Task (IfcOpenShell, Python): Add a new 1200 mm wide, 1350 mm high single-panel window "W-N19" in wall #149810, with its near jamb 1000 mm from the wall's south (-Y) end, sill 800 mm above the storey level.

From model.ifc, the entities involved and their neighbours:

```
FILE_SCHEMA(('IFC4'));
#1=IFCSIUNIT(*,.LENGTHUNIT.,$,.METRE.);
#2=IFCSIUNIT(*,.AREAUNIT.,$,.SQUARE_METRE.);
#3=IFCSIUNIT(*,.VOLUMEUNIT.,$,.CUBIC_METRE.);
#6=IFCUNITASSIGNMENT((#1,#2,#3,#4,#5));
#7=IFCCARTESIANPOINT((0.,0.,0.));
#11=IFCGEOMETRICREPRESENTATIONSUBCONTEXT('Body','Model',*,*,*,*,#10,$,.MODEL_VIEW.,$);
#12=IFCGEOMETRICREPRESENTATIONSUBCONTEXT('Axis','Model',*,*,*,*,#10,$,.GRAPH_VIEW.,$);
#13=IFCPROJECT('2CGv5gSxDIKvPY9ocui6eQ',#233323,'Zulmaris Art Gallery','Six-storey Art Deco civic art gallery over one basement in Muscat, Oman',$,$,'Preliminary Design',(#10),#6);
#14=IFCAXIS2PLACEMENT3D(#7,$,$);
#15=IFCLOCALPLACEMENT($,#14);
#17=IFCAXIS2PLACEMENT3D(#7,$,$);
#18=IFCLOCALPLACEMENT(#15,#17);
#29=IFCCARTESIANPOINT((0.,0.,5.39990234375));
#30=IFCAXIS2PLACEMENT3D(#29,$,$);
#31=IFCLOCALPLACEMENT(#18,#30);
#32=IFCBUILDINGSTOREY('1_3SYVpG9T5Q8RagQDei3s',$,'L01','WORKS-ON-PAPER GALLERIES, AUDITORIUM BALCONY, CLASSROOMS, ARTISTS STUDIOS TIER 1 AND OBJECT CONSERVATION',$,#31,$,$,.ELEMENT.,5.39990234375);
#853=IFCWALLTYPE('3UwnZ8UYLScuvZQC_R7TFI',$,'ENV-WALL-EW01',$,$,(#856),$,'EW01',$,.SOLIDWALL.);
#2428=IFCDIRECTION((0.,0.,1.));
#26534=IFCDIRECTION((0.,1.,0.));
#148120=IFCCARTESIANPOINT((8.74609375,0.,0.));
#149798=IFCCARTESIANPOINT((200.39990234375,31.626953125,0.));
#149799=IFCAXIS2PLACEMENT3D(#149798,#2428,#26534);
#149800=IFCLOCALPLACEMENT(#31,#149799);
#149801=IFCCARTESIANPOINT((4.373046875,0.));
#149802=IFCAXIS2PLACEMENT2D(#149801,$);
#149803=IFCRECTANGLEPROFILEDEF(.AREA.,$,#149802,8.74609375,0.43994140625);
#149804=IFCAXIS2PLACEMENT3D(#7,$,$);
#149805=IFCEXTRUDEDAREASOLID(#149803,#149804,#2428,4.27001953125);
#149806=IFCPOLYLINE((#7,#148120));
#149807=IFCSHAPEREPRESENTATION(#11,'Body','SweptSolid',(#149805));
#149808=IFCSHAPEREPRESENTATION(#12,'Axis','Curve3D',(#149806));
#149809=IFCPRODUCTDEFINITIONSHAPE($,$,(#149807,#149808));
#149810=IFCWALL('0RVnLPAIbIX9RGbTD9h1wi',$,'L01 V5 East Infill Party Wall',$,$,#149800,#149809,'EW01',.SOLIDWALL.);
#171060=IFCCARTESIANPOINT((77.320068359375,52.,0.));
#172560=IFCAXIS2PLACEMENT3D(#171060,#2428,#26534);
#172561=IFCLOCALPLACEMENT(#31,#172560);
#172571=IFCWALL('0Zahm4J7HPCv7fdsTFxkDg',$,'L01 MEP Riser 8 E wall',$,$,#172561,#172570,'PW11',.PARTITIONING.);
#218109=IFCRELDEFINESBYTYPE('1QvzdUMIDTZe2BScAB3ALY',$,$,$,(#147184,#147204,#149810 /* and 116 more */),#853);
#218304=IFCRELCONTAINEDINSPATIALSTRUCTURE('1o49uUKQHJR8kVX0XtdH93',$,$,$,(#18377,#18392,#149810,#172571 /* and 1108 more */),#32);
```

```python
import numpy as np
import ifcopenshell
import ifcopenshell.api.feature
import ifcopenshell.api.geometry
import ifcopenshell.api.root
import ifcopenshell.api.spatial
import ifcopenshell.geom
import ifcopenshell.util.element
import ifcopenshell.util.placement
import ifcopenshell.util.representation
import ifcopenshell.util.shape
import ifcopenshell.util.unit

model = ifcopenshell.open("model.ifc")
unit_scale = ifcopenshell.util.unit.calculate_unit_scale(model)
settings = ifcopenshell.geom.settings()


def volume(element):
    """Net volume in cubic metres, openings subtracted."""
    shape = ifcopenshell.geom.create_shape(settings, element)
    return ifcopenshell.util.shape.get_volume(shape.geometry)


wall = model.by_id(149810)
storey = ifcopenshell.util.element.get_container(wall, ifc_class="IfcBuildingStorey")
context = ifcopenshell.util.representation.get_context(model, "Model", "Body", "MODEL_VIEW")
before = volume(wall)

width, height, from_end, sill = 1.2, 1.35, 1, 0.8  # metres

# The wall runs along its own X axis, and the end named is its -X end.
wall_shape = ifcopenshell.geom.create_shape(settings, wall)
x, y, z = ifcopenshell.util.shape.get_vertices(wall_shape.geometry).T
start = x.min() + from_end
face, thickness = float(y.min()), float(y.max() - y.min())
wall_matrix = ifcopenshell.util.placement.get_local_placement(wall.ObjectPlacement)
level = ifcopenshell.util.placement.get_local_placement(storey.ObjectPlacement)[2, 3]


def in_wall(x, y):
    """Placement at x, y metres in the wall's axes, at sill height."""
    matrix = wall_matrix.copy()
    matrix[:, 3] = wall_matrix @ np.array([x / unit_scale, y / unit_scale, 0.0, 1.0])
    matrix[2, 3] = level + sill / unit_scale
    return matrix


# Opening: a box that overshoots both wall faces by 50 mm.
opening = ifcopenshell.api.root.create_entity(model, ifc_class="IfcOpeningElement", predefined_type="OPENING")
box = ifcopenshell.api.geometry.add_wall_representation(
    model, context=context, length=width, height=height, thickness=thickness + 0.1
)
ifcopenshell.api.geometry.assign_representation(model, product=opening, representation=box)
ifcopenshell.api.geometry.edit_object_placement(model, product=opening, matrix=in_wall(start, face - 0.05), is_si=False)
ifcopenshell.api.feature.add_feature(model, feature=opening, element=wall)

window = ifcopenshell.api.root.create_entity(model, ifc_class="IfcWindow", name="W-N19", predefined_type="WINDOW")
window.OverallWidth, window.OverallHeight = width / unit_scale, height / unit_scale
window.PartitioningType = "SINGLE_PANEL"
body = ifcopenshell.api.geometry.add_window_representation(
    model,
    context=context,
    overall_width=window.OverallWidth,
    overall_height=window.OverallHeight,
    partition_type="SINGLE_PANEL",
)
ifcopenshell.api.geometry.assign_representation(model, product=window, representation=body)
ifcopenshell.api.spatial.assign_container(model, products=[window], relating_structure=storey)
ifcopenshell.api.feature.add_filling(model, opening=opening, element=window)

# Centre the window in the wall's thickness.
ifcopenshell.api.geometry.edit_object_placement(model, product=window, matrix=in_wall(start, face), is_si=False)
window_shape = ifcopenshell.geom.create_shape(settings, window)
depth = ifcopenshell.util.shape.get_vertices(window_shape.geometry)[:, 1]
offset = face + thickness / 2 - (depth.min() + depth.max()) / 2
ifcopenshell.api.geometry.edit_object_placement(model, product=window, matrix=in_wall(start, offset), is_si=False)

after = volume(wall)

print(f"wall volume {before:.3f} -> {after:.3f} m3")

model.write("model_updated.ifc")
```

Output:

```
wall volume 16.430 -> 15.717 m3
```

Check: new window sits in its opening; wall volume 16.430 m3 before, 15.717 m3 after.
